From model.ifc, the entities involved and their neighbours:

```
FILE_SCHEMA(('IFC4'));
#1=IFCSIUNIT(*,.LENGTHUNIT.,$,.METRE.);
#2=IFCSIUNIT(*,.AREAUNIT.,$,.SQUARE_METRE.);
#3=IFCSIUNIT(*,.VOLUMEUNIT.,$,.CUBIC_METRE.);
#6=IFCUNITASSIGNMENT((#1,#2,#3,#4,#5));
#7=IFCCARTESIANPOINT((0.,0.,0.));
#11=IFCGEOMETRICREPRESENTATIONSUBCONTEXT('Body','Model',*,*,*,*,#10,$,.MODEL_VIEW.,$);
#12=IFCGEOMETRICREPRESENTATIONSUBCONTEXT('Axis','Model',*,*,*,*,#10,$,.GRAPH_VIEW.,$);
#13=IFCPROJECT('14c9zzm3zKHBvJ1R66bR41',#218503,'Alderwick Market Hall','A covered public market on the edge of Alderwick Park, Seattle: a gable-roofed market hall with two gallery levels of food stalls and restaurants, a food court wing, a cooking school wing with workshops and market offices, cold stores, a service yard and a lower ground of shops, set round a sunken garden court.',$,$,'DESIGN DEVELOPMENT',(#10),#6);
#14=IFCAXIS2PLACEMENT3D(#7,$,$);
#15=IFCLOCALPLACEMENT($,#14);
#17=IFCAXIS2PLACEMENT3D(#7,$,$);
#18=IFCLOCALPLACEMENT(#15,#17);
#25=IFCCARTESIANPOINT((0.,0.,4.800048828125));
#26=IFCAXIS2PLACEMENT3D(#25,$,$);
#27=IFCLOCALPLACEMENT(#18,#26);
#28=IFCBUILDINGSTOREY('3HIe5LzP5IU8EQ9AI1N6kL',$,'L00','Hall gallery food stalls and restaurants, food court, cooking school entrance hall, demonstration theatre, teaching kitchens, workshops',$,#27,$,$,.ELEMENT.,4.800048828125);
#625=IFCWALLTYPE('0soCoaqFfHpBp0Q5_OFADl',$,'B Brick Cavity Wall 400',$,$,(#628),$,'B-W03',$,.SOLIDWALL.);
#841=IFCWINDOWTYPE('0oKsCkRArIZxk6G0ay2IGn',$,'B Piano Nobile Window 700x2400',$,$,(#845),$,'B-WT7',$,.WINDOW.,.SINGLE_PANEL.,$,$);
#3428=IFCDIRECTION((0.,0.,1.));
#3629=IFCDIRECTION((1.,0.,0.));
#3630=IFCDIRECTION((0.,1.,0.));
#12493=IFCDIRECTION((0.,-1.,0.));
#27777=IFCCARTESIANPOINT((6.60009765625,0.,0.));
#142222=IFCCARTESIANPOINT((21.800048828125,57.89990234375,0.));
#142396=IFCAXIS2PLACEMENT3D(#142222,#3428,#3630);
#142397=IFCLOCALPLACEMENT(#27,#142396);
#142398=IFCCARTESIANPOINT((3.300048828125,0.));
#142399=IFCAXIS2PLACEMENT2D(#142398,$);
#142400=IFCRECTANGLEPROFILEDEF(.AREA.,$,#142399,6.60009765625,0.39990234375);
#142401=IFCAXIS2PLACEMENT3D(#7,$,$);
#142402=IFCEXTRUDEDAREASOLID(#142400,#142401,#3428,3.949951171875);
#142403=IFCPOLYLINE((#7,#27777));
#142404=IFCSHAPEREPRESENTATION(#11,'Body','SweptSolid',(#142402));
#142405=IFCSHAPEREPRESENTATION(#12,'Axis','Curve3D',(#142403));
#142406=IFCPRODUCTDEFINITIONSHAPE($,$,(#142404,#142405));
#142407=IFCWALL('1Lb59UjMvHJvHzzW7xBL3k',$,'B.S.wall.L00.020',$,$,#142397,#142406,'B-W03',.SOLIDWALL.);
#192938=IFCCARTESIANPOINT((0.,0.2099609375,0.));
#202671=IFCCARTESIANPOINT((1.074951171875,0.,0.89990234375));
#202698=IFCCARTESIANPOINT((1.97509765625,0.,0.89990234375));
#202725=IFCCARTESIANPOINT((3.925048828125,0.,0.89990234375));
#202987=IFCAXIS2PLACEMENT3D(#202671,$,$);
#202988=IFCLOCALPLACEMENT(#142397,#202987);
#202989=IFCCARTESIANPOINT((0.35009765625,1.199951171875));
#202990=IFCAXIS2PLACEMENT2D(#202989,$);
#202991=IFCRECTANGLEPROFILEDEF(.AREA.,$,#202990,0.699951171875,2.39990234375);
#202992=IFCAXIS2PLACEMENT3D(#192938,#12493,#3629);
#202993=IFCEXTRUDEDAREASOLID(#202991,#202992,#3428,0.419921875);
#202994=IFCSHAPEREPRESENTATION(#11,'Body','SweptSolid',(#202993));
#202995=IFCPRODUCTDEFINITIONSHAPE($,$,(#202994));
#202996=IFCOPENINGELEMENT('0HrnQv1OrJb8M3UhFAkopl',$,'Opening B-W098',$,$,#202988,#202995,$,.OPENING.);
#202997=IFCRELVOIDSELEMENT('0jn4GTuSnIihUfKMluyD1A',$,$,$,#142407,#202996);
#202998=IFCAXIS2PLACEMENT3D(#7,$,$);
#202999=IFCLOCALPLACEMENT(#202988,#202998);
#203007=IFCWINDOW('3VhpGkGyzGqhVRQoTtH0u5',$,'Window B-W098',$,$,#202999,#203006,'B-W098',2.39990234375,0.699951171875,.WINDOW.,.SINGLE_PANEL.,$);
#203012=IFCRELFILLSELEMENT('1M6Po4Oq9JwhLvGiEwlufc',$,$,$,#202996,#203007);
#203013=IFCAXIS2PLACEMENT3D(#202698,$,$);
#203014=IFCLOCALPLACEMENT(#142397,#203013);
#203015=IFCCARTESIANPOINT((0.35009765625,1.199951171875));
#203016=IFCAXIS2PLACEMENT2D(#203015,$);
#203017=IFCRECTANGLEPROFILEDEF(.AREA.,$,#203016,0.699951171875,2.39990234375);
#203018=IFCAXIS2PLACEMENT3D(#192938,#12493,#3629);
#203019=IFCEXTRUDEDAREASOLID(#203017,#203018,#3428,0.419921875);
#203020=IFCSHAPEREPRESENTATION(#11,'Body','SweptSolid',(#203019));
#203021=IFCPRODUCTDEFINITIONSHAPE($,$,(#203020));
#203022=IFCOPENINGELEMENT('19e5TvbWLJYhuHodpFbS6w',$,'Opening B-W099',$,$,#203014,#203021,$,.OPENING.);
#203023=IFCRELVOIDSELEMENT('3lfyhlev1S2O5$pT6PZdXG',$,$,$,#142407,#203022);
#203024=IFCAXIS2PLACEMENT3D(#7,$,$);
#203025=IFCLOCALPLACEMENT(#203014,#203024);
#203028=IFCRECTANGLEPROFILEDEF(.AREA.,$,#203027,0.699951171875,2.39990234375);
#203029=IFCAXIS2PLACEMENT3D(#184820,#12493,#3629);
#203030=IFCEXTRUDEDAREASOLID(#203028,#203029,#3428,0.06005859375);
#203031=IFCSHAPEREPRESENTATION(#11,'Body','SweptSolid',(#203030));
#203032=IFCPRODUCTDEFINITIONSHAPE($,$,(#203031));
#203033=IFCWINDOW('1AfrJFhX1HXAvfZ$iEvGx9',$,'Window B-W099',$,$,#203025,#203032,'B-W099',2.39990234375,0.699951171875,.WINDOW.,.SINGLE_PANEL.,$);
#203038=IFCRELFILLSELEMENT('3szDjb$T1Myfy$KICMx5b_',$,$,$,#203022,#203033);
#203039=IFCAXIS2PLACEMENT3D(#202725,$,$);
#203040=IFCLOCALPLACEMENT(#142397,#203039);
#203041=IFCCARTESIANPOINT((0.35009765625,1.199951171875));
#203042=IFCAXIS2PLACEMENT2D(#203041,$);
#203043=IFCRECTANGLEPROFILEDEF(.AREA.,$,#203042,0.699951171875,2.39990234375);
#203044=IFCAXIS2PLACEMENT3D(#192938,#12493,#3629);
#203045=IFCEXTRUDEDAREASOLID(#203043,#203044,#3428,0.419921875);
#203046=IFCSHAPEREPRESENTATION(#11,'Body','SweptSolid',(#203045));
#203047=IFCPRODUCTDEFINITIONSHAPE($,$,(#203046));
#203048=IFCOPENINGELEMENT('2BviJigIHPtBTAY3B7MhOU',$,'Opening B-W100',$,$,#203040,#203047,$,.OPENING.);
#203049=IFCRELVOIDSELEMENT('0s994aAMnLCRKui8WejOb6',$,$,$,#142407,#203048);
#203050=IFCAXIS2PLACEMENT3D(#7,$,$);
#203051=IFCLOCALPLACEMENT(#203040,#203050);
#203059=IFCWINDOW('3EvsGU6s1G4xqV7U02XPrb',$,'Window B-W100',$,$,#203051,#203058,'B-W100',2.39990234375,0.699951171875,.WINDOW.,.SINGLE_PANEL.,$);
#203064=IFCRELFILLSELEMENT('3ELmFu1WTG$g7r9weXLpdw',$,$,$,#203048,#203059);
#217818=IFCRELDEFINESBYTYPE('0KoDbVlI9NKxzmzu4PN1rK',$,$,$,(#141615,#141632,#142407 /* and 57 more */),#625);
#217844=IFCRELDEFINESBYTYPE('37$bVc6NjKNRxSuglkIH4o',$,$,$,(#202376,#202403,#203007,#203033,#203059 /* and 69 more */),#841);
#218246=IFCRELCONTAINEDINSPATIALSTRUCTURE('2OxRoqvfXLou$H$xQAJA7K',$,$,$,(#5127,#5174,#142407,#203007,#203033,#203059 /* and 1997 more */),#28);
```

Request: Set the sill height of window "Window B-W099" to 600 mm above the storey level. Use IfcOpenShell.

```python
import numpy as np
import ifcopenshell
import ifcopenshell.api.geometry
import ifcopenshell.geom
import ifcopenshell.util.element
import ifcopenshell.util.placement
import ifcopenshell.util.shape
import ifcopenshell.util.unit

model = ifcopenshell.open("model.ifc")
unit_scale = ifcopenshell.util.unit.calculate_unit_scale(model)

window = model.by_guid("1AfrJFhX1HXAvfZ$iEvGx9")
opening = window.FillsVoids[0].RelatingOpeningElement
storey = ifcopenshell.util.element.get_container(window, ifc_class="IfcBuildingStorey")
level = ifcopenshell.util.placement.get_local_placement(storey.ObjectPlacement)[2, 3]

# The opening's origin need not be at the sill, so measure its lowest point.
shape = ifcopenshell.geom.create_shape(ifcopenshell.geom.settings(), opening)
bottom = ifcopenshell.util.shape.get_shape_bottom_elevation(shape, shape.geometry) / unit_scale
dz = level + 0.6 / unit_scale - bottom

shift = np.array([0.0, 0.0, dz])
# The window is placed relative to its opening, so it follows when the opening moves.
matrix = ifcopenshell.util.placement.get_local_placement(opening.ObjectPlacement)
matrix[:3, 3] += shift
ifcopenshell.api.geometry.edit_object_placement(
    model, product=opening, matrix=matrix, is_si=False, should_transform_children=True
)

print(f"moved by {dz * unit_scale:+.3f} m")

model.write("model_rev.ifc")
```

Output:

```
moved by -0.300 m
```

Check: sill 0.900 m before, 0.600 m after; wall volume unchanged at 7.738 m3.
